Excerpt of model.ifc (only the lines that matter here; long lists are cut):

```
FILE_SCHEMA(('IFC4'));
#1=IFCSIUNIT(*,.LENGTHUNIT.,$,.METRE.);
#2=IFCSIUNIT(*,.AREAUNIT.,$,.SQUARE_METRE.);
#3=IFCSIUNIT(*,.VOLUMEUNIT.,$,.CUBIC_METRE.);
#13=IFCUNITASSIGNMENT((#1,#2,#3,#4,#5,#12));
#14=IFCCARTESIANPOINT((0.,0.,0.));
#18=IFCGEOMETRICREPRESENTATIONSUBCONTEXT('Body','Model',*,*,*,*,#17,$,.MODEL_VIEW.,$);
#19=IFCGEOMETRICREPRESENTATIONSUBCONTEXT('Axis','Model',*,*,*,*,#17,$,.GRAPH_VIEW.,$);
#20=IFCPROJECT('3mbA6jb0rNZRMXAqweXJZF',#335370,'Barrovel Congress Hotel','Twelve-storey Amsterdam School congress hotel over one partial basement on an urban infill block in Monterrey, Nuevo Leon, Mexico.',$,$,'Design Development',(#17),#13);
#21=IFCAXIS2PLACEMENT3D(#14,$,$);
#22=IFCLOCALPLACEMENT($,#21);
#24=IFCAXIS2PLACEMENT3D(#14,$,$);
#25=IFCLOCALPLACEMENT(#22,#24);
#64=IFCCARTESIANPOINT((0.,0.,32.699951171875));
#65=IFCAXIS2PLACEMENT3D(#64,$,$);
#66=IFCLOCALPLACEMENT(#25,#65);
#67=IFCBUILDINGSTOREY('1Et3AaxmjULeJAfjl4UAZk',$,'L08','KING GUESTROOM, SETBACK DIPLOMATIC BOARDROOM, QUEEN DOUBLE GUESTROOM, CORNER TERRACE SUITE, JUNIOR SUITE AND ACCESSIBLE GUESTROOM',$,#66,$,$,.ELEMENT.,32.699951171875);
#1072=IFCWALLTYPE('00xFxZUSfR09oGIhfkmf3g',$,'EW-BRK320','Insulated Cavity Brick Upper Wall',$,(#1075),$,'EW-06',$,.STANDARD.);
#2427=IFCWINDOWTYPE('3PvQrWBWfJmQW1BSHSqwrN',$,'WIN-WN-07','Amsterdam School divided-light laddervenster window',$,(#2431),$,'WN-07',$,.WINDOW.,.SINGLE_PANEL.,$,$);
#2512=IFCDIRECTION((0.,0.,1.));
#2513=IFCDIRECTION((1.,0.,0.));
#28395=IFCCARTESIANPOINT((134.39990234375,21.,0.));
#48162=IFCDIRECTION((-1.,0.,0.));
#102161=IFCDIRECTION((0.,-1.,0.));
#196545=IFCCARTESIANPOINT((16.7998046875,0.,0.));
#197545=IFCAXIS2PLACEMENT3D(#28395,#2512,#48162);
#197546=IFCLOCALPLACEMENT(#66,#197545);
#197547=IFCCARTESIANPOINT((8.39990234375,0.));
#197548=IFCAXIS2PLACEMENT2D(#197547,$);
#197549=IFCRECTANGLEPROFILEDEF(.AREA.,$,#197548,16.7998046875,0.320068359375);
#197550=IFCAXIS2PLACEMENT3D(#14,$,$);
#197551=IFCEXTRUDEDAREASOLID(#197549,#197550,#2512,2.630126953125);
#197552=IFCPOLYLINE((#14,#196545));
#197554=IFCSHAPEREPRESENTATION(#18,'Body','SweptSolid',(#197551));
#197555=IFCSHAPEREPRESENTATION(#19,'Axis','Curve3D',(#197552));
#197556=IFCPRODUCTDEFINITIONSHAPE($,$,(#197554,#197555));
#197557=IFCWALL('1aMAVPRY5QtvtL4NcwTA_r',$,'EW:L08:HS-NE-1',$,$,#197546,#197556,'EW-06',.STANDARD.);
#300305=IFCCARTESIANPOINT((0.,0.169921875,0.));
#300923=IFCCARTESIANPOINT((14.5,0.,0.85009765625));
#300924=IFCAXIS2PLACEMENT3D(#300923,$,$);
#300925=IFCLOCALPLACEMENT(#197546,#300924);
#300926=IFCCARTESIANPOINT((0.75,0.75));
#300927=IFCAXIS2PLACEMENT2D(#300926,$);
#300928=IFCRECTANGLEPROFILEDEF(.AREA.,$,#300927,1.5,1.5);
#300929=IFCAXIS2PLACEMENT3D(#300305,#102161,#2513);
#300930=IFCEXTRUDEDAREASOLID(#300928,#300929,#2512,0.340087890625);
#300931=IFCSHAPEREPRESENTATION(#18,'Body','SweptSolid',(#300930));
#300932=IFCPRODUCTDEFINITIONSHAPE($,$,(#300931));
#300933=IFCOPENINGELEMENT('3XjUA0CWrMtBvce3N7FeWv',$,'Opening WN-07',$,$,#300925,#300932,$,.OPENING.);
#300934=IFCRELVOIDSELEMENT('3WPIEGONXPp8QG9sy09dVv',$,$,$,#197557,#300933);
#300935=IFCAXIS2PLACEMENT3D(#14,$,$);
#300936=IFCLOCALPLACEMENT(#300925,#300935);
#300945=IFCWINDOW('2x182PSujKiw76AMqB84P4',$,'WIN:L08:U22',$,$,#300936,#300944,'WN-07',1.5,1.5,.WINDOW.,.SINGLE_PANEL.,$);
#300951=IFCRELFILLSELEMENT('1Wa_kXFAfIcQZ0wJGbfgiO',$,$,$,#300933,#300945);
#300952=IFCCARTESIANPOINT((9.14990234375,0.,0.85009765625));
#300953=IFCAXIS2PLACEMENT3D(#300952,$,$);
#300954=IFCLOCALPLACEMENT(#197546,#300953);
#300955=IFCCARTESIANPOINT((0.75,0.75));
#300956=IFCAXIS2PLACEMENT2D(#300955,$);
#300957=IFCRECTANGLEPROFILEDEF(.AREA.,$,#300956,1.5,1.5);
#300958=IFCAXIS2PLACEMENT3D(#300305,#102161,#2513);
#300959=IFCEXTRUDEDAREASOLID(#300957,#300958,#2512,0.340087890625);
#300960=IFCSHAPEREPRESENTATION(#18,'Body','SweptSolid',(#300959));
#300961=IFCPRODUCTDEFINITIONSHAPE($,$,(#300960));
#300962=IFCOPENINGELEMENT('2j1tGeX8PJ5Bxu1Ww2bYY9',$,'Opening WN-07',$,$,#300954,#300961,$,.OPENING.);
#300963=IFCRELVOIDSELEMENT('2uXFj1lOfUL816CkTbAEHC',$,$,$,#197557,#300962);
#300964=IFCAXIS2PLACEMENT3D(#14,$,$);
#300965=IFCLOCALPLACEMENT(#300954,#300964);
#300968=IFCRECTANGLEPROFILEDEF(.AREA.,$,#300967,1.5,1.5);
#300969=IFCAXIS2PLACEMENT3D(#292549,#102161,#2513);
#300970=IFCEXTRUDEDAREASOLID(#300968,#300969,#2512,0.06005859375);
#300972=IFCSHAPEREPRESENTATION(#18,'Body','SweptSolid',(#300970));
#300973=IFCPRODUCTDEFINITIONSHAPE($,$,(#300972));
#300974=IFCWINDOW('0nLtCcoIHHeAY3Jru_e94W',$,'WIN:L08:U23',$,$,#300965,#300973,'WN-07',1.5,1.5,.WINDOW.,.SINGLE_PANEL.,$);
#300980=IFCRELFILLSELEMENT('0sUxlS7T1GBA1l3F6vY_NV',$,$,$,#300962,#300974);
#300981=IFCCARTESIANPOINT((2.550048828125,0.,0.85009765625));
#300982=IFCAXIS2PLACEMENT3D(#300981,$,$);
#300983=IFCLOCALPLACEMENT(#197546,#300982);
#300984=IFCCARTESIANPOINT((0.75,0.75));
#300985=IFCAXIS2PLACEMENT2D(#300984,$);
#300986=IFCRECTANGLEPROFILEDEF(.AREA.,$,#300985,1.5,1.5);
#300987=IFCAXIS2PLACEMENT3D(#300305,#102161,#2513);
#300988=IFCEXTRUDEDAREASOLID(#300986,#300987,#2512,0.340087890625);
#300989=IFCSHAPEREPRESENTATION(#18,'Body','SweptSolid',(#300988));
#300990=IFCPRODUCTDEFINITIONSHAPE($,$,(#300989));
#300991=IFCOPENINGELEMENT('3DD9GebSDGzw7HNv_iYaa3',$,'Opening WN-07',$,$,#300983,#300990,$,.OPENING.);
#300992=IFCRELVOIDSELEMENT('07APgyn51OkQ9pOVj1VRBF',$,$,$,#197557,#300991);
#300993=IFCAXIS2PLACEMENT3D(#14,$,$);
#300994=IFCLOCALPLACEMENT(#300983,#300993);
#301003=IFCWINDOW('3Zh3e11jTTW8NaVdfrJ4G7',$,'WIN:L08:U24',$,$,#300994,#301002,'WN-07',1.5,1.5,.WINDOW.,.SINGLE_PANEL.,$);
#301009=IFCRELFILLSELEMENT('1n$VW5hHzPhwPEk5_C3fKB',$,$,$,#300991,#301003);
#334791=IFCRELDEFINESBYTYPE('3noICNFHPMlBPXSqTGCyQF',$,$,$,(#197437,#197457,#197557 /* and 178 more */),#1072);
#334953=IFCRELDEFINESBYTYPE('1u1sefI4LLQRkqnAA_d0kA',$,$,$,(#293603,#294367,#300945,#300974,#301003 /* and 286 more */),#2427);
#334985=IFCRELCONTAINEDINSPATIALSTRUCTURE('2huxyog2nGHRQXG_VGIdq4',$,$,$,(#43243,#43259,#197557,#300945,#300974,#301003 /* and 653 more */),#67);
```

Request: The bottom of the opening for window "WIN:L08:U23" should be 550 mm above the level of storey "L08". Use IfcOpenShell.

```python
import numpy as np
import ifcopenshell
import ifcopenshell.api.geometry
import ifcopenshell.geom
import ifcopenshell.util.element
import ifcopenshell.util.placement
import ifcopenshell.util.shape
import ifcopenshell.util.unit

model = ifcopenshell.open("model.ifc")
unit_scale = ifcopenshell.util.unit.calculate_unit_scale(model)

window = model.by_guid("0nLtCcoIHHeAY3Jru_e94W")
opening = window.FillsVoids[0].RelatingOpeningElement
storey = ifcopenshell.util.element.get_container(window, ifc_class="IfcBuildingStorey")
level = ifcopenshell.util.placement.get_local_placement(storey.ObjectPlacement)[2, 3]

# The opening's origin need not be at the sill, so measure its lowest point.
shape = ifcopenshell.geom.create_shape(ifcopenshell.geom.settings(), opening)
bottom = ifcopenshell.util.shape.get_shape_bottom_elevation(shape, shape.geometry) / unit_scale
dz = level + 0.55 - bottom

shift = np.array([0.0, 0.0, dz])
# The window is placed relative to its opening, so it follows when the opening moves.
matrix = ifcopenshell.util.placement.get_local_placement(opening.ObjectPlacement)
matrix[:3, 3] += shift
ifcopenshell.api.geometry.edit_object_placement(
    model, product=opening, matrix=matrix, is_si=False, should_transform_children=True
)

print(f"moved by {dz * unit_scale:+.3f} m")

model.write("model_rev.ifc")
```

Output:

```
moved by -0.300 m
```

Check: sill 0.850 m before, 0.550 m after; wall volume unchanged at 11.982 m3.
